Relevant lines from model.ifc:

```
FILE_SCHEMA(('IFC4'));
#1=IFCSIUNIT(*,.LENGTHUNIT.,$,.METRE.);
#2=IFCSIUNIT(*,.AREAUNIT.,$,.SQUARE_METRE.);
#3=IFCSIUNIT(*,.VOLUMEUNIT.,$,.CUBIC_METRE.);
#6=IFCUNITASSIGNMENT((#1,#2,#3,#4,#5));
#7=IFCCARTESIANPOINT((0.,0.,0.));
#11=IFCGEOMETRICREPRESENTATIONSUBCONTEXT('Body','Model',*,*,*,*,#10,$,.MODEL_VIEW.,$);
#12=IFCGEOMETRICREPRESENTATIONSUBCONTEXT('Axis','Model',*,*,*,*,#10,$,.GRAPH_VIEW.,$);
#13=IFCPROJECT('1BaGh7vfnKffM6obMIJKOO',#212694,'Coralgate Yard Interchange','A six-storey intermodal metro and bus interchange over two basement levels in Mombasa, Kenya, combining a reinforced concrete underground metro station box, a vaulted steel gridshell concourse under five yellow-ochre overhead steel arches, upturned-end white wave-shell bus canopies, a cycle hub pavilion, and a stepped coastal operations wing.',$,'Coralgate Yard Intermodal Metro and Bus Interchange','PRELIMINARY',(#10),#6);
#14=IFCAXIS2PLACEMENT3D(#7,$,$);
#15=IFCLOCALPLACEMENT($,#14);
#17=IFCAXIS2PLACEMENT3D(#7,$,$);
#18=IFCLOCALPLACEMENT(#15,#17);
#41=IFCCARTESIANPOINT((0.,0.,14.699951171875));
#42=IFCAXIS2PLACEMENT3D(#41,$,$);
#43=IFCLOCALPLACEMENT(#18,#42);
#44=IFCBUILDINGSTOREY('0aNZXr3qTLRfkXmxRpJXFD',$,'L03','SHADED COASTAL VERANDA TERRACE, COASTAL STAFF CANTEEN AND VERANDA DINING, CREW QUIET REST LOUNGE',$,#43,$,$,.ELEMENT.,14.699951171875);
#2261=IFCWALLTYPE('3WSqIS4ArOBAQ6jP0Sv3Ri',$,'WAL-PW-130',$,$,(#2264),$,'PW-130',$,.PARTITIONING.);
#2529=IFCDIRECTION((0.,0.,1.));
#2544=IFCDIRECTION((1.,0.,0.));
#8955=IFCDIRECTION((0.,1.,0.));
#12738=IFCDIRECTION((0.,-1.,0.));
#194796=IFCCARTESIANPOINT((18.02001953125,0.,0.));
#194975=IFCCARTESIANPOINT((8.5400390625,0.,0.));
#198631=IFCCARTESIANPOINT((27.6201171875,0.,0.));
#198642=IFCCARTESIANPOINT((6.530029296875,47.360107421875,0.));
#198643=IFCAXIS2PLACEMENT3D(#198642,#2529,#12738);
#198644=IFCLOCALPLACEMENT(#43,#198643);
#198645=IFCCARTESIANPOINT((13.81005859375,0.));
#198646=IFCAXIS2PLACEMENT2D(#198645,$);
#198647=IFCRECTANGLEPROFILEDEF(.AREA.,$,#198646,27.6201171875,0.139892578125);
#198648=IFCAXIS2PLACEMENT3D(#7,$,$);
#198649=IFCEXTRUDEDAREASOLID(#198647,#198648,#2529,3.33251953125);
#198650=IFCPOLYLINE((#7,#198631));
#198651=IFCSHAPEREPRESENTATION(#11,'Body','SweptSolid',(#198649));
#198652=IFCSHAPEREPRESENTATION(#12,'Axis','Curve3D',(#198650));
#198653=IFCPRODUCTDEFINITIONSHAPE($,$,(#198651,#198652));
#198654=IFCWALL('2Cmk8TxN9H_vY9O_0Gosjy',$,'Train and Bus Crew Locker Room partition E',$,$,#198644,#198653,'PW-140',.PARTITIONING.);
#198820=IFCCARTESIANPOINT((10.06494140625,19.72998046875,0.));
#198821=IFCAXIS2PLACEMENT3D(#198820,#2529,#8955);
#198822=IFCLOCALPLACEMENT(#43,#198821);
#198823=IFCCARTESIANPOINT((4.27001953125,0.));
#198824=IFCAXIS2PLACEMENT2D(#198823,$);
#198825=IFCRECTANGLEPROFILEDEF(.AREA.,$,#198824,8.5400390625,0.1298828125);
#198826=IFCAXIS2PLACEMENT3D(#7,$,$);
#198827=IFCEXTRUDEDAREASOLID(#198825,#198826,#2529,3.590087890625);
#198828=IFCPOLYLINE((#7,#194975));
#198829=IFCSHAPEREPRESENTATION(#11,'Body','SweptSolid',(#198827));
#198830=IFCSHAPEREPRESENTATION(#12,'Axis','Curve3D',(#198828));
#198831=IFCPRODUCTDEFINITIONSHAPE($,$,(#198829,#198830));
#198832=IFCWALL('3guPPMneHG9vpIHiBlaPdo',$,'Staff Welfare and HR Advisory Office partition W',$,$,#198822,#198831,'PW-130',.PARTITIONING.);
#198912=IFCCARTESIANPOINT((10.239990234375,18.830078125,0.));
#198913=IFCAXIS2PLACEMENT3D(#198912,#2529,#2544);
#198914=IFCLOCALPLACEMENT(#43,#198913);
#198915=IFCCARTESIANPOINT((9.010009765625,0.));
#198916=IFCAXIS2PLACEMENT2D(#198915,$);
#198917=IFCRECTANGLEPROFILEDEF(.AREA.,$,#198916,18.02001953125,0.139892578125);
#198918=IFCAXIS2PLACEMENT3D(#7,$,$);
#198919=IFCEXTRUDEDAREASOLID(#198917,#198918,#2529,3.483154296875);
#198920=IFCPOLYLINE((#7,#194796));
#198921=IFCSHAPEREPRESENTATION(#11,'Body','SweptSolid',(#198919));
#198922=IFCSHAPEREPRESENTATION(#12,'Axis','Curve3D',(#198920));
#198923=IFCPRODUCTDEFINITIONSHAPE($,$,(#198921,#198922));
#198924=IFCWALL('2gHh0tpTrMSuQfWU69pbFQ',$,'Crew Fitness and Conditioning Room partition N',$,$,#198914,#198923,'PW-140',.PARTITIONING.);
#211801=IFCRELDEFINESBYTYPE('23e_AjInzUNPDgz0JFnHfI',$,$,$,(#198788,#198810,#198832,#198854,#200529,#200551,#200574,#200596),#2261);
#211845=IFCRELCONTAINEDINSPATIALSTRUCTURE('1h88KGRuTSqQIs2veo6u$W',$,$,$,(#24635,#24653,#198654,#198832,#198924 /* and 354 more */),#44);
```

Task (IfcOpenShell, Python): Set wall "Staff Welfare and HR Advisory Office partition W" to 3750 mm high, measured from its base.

```python
import ifcopenshell
import ifcopenshell.geom
import ifcopenshell.util.representation
import ifcopenshell.util.shape
import ifcopenshell.util.unit

model = ifcopenshell.open("model.ifc")
unit_scale = ifcopenshell.util.unit.calculate_unit_scale(model)
settings = ifcopenshell.geom.settings()


def volume(element):
    """Net volume in cubic metres, openings subtracted."""
    shape = ifcopenshell.geom.create_shape(settings, element)
    return ifcopenshell.util.shape.get_volume(shape.geometry)


wall = model.by_id(198832)
before = volume(wall)

body = ifcopenshell.util.representation.get_representation(wall, "Model", "Body")
solid = body.Items[0]
old_height = solid.Depth
solid.Depth = 3.75 / unit_scale
after = volume(wall)

print(f"height {old_height:g} -> {solid.Depth:g}, volume {before:.3f} -> {after:.3f} m3")

model.write("model-out.ifc")
```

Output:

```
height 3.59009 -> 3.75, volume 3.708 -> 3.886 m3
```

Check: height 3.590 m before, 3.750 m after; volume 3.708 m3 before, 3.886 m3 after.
